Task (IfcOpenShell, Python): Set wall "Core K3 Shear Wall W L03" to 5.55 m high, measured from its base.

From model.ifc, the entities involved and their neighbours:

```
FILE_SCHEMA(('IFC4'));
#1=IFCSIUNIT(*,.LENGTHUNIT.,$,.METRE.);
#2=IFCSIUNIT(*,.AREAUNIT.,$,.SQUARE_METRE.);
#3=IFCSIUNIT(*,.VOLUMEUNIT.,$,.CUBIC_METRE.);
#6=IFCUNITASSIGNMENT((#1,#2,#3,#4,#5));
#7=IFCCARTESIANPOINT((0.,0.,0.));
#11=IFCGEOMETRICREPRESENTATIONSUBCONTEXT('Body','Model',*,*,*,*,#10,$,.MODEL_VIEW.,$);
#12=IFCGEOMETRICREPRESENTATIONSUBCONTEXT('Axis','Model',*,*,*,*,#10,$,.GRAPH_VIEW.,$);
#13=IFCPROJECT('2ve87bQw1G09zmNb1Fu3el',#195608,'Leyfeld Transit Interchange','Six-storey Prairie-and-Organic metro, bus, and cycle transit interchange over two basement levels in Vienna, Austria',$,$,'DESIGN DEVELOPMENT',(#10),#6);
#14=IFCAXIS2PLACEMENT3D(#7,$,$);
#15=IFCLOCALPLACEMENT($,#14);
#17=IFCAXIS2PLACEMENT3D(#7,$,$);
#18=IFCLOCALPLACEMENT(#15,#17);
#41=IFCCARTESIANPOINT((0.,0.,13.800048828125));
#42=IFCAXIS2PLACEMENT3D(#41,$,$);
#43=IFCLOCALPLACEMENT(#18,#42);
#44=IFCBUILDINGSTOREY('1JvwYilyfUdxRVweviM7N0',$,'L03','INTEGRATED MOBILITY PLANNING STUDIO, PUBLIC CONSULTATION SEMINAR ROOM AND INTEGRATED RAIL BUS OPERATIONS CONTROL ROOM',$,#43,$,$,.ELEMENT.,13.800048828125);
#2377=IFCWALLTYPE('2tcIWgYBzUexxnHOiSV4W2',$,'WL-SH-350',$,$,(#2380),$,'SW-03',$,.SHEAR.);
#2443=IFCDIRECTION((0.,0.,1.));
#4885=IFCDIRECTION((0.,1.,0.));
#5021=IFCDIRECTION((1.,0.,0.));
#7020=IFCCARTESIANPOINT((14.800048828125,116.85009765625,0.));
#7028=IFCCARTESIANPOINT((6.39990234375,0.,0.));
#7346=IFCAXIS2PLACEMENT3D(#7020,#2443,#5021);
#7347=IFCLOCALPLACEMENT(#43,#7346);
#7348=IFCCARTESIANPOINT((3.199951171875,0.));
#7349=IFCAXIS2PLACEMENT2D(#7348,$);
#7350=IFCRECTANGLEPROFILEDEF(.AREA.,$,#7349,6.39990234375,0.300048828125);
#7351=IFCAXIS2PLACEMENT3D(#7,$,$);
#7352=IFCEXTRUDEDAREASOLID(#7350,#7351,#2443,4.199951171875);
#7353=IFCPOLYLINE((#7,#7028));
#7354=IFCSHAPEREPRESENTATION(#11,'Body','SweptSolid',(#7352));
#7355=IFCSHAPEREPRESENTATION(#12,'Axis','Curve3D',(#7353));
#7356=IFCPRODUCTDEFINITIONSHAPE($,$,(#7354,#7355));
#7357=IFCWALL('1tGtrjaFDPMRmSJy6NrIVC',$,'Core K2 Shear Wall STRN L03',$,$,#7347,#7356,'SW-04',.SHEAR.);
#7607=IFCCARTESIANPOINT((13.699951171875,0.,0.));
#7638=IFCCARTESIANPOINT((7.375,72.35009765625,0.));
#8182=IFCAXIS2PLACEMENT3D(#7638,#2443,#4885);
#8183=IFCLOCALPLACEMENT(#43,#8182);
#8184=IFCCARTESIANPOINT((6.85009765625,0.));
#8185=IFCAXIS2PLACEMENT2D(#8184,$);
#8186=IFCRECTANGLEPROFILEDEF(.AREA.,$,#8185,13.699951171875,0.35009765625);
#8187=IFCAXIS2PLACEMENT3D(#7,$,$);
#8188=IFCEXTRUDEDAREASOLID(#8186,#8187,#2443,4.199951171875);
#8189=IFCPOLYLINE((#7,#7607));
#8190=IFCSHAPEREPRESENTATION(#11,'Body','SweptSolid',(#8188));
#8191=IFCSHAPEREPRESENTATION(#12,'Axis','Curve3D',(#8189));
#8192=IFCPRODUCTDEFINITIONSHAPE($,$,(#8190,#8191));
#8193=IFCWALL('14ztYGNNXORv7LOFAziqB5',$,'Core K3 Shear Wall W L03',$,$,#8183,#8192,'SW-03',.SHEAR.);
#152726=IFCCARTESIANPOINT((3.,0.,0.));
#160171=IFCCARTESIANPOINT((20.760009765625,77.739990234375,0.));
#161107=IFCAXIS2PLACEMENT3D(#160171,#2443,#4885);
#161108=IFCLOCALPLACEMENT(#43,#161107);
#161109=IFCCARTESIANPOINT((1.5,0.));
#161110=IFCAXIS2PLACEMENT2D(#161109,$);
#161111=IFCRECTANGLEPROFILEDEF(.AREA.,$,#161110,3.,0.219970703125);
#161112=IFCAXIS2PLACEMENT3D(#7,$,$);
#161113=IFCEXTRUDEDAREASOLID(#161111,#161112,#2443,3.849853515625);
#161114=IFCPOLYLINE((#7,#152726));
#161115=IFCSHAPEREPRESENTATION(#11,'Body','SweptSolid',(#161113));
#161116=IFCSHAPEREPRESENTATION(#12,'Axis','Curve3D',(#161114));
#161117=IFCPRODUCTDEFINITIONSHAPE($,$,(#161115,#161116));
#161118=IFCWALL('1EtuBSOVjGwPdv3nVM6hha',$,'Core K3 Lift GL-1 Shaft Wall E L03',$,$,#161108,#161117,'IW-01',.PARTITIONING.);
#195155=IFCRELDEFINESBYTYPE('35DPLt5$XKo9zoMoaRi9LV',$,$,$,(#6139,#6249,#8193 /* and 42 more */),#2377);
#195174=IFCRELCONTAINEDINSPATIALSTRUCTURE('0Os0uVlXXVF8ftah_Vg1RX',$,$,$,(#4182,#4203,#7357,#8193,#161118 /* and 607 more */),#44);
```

```python
import ifcopenshell
import ifcopenshell.geom
import ifcopenshell.util.representation
import ifcopenshell.util.shape
import ifcopenshell.util.unit

model = ifcopenshell.open("model.ifc")
unit_scale = ifcopenshell.util.unit.calculate_unit_scale(model)
settings = ifcopenshell.geom.settings()


def volume(element):
    """Net volume in cubic metres, openings subtracted."""
    shape = ifcopenshell.geom.create_shape(settings, element)
    return ifcopenshell.util.shape.get_volume(shape.geometry)


wall = model.by_guid("14ztYGNNXORv7LOFAziqB5")
before = volume(wall)

body = ifcopenshell.util.representation.get_representation(wall, "Model", "Body")
solid = body.Items[0]
old_height = solid.Depth
solid.Depth = 5.55 / unit_scale
after = volume(wall)

print(f"height {old_height:g} -> {solid.Depth:g}, volume {before:.3f} -> {after:.3f} m3")

model.write("model_rev.ifc")
```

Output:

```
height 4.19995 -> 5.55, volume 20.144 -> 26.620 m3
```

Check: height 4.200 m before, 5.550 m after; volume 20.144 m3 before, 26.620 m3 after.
